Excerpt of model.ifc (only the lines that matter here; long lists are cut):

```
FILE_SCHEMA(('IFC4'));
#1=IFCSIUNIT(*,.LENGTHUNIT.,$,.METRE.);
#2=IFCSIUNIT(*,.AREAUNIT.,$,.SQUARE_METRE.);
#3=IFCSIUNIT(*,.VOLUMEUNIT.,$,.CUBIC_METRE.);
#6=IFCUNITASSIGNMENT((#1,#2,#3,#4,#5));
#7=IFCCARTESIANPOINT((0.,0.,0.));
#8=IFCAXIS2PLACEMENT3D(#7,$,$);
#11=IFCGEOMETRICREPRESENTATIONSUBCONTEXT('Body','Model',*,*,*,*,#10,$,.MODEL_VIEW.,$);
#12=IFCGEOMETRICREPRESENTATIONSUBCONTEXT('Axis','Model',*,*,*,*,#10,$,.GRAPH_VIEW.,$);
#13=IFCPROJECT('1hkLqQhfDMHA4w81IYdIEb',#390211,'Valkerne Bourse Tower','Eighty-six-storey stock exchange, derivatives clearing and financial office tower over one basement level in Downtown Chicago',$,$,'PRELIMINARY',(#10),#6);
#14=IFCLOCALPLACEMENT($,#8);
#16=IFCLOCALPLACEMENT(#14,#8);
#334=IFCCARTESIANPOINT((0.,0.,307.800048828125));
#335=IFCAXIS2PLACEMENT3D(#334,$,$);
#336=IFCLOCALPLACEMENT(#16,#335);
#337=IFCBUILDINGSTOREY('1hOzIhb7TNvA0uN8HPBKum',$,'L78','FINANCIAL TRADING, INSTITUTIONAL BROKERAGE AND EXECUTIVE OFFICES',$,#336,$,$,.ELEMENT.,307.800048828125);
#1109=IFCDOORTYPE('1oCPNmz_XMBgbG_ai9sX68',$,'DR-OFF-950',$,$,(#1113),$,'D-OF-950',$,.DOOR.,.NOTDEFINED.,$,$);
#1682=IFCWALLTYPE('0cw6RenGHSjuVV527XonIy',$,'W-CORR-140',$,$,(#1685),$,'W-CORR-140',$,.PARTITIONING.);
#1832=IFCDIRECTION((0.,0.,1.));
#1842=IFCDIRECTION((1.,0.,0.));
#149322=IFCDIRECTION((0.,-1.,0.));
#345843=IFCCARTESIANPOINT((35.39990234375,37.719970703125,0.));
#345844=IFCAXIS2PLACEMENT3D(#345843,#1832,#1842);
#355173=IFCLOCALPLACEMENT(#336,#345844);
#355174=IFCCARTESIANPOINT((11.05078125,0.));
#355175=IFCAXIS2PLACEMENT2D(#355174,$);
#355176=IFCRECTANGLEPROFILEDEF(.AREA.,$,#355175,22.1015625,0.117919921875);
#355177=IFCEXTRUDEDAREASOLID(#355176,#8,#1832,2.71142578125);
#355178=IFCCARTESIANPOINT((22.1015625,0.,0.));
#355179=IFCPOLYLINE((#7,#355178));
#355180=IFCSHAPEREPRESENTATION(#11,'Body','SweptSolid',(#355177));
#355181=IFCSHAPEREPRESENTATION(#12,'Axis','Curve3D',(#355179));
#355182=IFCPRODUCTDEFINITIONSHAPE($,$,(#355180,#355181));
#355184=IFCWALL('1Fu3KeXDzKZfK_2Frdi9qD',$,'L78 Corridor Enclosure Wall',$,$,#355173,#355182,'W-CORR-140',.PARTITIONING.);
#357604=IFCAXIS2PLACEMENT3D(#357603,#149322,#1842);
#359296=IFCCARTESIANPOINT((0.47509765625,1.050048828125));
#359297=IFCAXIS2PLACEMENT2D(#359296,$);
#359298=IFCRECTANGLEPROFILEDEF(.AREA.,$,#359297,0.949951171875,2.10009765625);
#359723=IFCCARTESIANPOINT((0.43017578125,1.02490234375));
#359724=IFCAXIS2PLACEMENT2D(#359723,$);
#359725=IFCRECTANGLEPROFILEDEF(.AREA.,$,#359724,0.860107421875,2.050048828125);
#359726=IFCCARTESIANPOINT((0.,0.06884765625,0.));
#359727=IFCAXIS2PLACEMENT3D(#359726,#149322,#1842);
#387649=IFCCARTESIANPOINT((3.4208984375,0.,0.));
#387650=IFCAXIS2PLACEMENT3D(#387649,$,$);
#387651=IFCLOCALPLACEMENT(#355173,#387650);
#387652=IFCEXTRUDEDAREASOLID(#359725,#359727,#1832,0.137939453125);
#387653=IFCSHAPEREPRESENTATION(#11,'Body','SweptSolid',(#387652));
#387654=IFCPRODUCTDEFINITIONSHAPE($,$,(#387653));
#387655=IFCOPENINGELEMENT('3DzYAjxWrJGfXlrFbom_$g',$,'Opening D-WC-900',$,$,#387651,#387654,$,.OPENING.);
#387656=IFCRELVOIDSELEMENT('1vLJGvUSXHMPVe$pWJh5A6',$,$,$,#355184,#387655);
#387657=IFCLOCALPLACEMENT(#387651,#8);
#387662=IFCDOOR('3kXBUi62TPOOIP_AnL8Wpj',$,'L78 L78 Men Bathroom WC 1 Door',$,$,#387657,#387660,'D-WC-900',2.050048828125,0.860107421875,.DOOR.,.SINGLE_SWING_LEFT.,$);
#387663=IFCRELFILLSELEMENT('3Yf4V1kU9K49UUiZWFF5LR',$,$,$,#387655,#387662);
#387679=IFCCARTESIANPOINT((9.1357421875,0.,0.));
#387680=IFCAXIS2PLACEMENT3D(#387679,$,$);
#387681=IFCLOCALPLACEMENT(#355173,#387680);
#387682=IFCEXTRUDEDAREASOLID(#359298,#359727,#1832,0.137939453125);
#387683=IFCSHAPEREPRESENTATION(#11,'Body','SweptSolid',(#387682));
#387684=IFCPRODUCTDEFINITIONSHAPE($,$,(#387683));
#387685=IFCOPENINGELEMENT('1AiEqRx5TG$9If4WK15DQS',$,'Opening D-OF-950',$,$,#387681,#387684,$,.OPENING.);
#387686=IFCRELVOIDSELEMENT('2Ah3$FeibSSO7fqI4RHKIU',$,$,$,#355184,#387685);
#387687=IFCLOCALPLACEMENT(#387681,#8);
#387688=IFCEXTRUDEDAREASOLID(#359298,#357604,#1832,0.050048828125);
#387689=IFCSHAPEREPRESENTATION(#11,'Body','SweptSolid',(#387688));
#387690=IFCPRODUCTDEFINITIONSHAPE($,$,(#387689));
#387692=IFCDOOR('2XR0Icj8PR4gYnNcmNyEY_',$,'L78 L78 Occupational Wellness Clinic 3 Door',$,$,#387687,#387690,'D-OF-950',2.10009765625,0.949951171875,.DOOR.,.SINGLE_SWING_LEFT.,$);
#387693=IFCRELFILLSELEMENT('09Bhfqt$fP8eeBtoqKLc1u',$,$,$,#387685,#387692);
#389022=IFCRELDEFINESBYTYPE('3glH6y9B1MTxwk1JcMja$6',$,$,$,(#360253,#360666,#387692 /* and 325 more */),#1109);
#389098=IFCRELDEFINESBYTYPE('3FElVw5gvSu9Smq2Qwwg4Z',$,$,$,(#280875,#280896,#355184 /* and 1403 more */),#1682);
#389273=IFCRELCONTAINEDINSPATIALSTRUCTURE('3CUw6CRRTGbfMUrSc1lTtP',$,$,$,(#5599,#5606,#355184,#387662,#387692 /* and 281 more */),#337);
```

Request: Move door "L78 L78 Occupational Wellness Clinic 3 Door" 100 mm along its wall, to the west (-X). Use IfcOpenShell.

```python
import ifcopenshell
import ifcopenshell.api.geometry
import ifcopenshell.util.placement

model = ifcopenshell.open("model.ifc")

door = model.by_guid("2XR0Icj8PR4gYnNcmNyEY_")
opening = door.FillsVoids[0].RelatingOpeningElement
wall = opening.VoidsElements[0].RelatingBuildingElement

wall_matrix = ifcopenshell.util.placement.get_local_placement(wall.ObjectPlacement)
shift = wall_matrix[:3, 0] * -0.1
before = ifcopenshell.util.placement.get_local_placement(door.ObjectPlacement)[:3, 3].copy()

# The door is placed relative to its opening, so it follows when the opening moves.
matrix = ifcopenshell.util.placement.get_local_placement(opening.ObjectPlacement)
matrix[:3, 3] += shift
ifcopenshell.api.geometry.edit_object_placement(
    model, product=opening, matrix=matrix, is_si=False, should_transform_children=True
)

after = ifcopenshell.util.placement.get_local_placement(door.ObjectPlacement)[:3, 3]
print("door moved by", (after - before).round(3) + 0.0)

model.write("model_updated.ifc")
```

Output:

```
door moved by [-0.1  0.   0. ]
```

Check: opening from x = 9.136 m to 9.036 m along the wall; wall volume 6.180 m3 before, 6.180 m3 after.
